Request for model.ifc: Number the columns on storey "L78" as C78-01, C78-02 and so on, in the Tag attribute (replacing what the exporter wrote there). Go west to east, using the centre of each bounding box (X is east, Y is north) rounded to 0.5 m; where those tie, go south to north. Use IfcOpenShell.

First a look at what the model holds.

```python
import ifcopenshell
import ifcopenshell.util.element
import ifcopenshell.util.placement

model = ifcopenshell.open("model.ifc")
print(model.schema)
storey = next(s for s in model.by_type("IfcBuildingStorey") if s.Name == "L78")
columns = [e for e in ifcopenshell.util.element.get_decomposition(storey) if e.is_a("IfcColumn")]
for e in sorted(columns, key=lambda e: e.id()):
    origin = ifcopenshell.util.placement.get_local_placement(e.ObjectPlacement)[:3, 3]
    print(e.id(), e.Tag, e.Name, origin.round(2) + 0.0, sep=" | ")
```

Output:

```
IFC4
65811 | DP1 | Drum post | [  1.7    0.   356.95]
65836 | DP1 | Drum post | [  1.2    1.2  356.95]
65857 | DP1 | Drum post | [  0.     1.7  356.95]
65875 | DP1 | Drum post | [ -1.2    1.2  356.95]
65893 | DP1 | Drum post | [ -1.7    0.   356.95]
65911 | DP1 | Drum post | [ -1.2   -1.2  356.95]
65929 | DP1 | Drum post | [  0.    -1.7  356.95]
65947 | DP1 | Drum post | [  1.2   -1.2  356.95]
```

```python
import ifcopenshell
import ifcopenshell.geom
import ifcopenshell.util.element
import ifcopenshell.util.shape

model = ifcopenshell.open("model.ifc")
settings = ifcopenshell.geom.settings()
settings.set("use-world-coords", True)


def centre(element):
    shape = ifcopenshell.geom.create_shape(settings, element)
    return ifcopenshell.util.shape.get_bbox_centroid(shape.geometry)


storey = next(s for s in model.by_type("IfcBuildingStorey") if s.Name == "L78")
columns = [e for e in ifcopenshell.util.element.get_decomposition(storey) if e.is_a("IfcColumn")]

# Insertion points can sit at a corner or the storey origin, so sort by the geometry (in metres).
centres = {e: centre(e) for e in columns}
columns.sort(key=lambda e: (round(centres[e][0] / 0.5), centres[e][1]))

for i, e in enumerate(columns, start=1):
    number = f"C78-{i:02d}"
    e.Tag = number
    print(e.id(), number)

model.write("model_rev.ifc")
```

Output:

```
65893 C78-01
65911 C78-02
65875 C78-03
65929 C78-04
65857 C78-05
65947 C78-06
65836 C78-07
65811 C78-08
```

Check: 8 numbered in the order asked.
